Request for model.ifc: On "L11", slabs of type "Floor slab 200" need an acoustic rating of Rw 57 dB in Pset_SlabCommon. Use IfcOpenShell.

First a look at what the model holds.

```python
import ifcopenshell
import ifcopenshell.util.element

model = ifcopenshell.open("model.ifc")
print(model.schema)
storey = next(s for s in model.by_type("IfcBuildingStorey") if s.Name == "L11")
slabs = [e for e in ifcopenshell.util.element.get_decomposition(storey) if e.is_a("IfcSlab")]
seen = {}
for e in slabs:
    element_type = ifcopenshell.util.element.get_type(e)
    key = (element_type.Name if element_type != e and element_type else None, ifcopenshell.util.element.get_pset(e, "Pset_SlabCommon", "AcousticRating"))
    seen[key] = seen.get(key, 0) + 1
for (name, value), count in sorted(seen.items(), key=str):
    print(count, "x", name, "|", value)
```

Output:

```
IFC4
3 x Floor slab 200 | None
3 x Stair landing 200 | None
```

```python
import ifcopenshell
import ifcopenshell.api.pset
import ifcopenshell.util.element

model = ifcopenshell.open("model.ifc")

storey = next(s for s in model.by_type("IfcBuildingStorey") if s.Name == "L11")
slabs = [e for e in ifcopenshell.util.element.get_decomposition(storey) if e.is_a("IfcSlab")]

count = 0
for e in slabs:
    element_type = ifcopenshell.util.element.get_type(e)
    if element_type in (None, e) or element_type.Name != "Floor slab 200":
        continue
    found = ifcopenshell.util.element.get_pset(e, "Pset_SlabCommon", should_inherit=False)
    if found:
        pset = model.by_id(found["id"])
        if len(ifcopenshell.util.element.get_elements_by_pset(pset)) > 1:
            pset = ifcopenshell.api.pset.unshare_pset(model, products=[e], pset=pset)[0]
    else:
        pset = ifcopenshell.api.pset.add_pset(model, product=e, name="Pset_SlabCommon")
    ifcopenshell.api.pset.edit_pset(model, pset=pset, properties={"AcousticRating": "Rw 57 dB"})
    count += 1

print(count, "slabs updated")

model.write("model_v2.ifc")
```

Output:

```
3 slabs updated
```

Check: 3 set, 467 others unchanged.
